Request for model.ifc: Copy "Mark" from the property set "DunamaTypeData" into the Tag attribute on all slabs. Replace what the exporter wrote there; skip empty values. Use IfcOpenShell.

First a look at what the model holds.

```python
import ifcopenshell
import ifcopenshell.util.element

model = ifcopenshell.open("model.ifc")
print(model.schema)
slabs = model.by_type("IfcSlab")
print(len(slabs), "slabs")
for e in slabs[:8]:
    source = ifcopenshell.util.element.get_pset(e, "DunamaTypeData", "Mark")
    target = e.Tag
    print(e.id(), repr(source), repr(target), sep=" | ")
```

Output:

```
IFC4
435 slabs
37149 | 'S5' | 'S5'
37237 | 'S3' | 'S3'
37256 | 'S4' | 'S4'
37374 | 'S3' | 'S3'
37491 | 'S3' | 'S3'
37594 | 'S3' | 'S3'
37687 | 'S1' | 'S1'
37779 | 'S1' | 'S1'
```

```python
import ifcopenshell
import ifcopenshell.util.element

model = ifcopenshell.open("model.ifc")

count = 0
for e in model.by_type("IfcSlab"):
    value = ifcopenshell.util.element.get_pset(e, "DunamaTypeData", "Mark")
    current = e.Tag
    if not value or not value.strip() or current == value:
        continue
    e.Tag = value
    count += 1

print(count, "slabs updated")

model.write("model_rev.ifc")
```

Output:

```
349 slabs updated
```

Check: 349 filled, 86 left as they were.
